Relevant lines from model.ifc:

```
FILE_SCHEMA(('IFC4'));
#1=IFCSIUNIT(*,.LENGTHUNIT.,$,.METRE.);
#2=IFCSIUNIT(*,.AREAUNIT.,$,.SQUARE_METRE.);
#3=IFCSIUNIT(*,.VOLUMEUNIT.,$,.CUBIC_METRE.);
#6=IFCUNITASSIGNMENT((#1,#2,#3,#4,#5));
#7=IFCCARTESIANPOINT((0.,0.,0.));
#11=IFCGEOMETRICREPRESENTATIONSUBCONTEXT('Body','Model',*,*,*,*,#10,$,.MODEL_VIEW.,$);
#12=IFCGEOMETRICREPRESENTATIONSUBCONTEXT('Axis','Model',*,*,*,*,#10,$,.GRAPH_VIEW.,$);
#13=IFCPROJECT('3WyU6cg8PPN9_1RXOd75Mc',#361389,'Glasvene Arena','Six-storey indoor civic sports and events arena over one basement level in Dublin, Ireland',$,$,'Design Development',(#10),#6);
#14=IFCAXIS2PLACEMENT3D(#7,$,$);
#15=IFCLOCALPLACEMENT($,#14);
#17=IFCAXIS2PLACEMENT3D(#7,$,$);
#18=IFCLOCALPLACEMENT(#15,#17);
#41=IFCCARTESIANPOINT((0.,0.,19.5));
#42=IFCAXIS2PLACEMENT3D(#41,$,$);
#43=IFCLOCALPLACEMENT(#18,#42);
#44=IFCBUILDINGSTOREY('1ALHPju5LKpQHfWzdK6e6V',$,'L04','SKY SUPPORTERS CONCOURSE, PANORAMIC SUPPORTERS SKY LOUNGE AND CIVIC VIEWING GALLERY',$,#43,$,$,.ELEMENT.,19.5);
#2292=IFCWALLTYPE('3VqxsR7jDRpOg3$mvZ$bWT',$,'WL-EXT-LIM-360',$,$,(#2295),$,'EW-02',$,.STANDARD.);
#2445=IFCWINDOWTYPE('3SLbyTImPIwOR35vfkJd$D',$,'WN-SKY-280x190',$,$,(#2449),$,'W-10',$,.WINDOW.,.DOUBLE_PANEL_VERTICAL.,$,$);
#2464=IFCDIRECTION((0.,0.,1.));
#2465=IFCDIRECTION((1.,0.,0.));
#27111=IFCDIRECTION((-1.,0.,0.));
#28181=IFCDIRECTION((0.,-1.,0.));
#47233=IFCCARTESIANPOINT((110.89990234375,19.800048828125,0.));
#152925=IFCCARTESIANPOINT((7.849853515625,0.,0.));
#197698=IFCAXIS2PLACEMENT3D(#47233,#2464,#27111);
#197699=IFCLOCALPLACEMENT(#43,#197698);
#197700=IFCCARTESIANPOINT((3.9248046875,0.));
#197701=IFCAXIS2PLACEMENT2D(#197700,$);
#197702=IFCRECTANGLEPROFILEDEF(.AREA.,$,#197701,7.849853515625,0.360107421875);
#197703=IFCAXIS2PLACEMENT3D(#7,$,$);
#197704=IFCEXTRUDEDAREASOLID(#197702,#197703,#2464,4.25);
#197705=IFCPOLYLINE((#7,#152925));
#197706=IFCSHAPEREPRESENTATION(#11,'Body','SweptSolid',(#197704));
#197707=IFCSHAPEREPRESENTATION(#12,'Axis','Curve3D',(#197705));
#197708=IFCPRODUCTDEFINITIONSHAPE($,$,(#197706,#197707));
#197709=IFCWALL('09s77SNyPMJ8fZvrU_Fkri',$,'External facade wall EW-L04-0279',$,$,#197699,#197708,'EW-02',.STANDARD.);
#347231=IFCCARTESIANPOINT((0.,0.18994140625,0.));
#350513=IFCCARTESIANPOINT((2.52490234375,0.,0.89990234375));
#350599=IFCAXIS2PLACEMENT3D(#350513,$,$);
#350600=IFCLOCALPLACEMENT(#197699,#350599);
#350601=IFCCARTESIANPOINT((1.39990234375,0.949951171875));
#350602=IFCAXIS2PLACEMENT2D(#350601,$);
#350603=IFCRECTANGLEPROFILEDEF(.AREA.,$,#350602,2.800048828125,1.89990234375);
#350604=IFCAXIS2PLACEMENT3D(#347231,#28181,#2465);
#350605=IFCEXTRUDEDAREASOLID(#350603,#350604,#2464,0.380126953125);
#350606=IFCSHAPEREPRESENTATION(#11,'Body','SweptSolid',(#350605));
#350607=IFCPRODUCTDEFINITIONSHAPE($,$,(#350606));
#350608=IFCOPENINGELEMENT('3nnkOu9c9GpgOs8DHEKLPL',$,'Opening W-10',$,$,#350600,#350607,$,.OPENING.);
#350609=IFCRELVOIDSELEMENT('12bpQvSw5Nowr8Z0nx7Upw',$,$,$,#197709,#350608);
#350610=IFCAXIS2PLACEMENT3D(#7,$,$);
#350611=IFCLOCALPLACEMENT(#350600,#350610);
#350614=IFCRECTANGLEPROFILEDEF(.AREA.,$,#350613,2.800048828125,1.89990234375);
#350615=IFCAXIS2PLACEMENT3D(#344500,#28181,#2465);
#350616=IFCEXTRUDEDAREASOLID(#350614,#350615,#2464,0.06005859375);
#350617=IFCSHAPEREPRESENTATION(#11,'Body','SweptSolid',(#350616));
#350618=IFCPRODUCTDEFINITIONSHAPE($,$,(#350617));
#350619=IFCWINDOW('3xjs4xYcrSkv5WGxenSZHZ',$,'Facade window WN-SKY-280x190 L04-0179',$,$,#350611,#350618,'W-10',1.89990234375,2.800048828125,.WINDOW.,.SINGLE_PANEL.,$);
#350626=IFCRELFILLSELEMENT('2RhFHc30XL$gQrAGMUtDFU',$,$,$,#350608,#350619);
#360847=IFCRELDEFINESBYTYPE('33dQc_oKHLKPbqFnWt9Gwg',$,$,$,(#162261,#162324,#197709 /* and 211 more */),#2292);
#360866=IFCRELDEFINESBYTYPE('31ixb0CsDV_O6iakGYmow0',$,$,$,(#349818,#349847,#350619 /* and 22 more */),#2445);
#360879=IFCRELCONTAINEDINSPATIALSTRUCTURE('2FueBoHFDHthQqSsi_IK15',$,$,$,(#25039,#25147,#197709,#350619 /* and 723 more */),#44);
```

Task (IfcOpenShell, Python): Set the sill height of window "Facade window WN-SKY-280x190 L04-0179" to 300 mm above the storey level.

```python
import numpy as np
import ifcopenshell
import ifcopenshell.api.geometry
import ifcopenshell.geom
import ifcopenshell.util.element
import ifcopenshell.util.placement
import ifcopenshell.util.shape
import ifcopenshell.util.unit

model = ifcopenshell.open("model.ifc")
unit_scale = ifcopenshell.util.unit.calculate_unit_scale(model)

window = model.by_id(350619)
opening = window.FillsVoids[0].RelatingOpeningElement
storey = ifcopenshell.util.element.get_container(window, ifc_class="IfcBuildingStorey")
level = ifcopenshell.util.placement.get_local_placement(storey.ObjectPlacement)[2, 3]

# The opening's origin need not be at the sill, so measure its lowest point.
shape = ifcopenshell.geom.create_shape(ifcopenshell.geom.settings(), opening)
bottom = ifcopenshell.util.shape.get_shape_bottom_elevation(shape, shape.geometry) / unit_scale
dz = level + 0.3 - bottom

shift = np.array([0.0, 0.0, dz])
# The window is placed relative to its opening, so it follows when the opening moves.
matrix = ifcopenshell.util.placement.get_local_placement(opening.ObjectPlacement)
matrix[:3, 3] += shift
ifcopenshell.api.geometry.edit_object_placement(
    model, product=opening, matrix=matrix, is_si=False, should_transform_children=True
)

print(f"moved by {dz * unit_scale:+.3f} m")

model.write("model-out.ifc")
```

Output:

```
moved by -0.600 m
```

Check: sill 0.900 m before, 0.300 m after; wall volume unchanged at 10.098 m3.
